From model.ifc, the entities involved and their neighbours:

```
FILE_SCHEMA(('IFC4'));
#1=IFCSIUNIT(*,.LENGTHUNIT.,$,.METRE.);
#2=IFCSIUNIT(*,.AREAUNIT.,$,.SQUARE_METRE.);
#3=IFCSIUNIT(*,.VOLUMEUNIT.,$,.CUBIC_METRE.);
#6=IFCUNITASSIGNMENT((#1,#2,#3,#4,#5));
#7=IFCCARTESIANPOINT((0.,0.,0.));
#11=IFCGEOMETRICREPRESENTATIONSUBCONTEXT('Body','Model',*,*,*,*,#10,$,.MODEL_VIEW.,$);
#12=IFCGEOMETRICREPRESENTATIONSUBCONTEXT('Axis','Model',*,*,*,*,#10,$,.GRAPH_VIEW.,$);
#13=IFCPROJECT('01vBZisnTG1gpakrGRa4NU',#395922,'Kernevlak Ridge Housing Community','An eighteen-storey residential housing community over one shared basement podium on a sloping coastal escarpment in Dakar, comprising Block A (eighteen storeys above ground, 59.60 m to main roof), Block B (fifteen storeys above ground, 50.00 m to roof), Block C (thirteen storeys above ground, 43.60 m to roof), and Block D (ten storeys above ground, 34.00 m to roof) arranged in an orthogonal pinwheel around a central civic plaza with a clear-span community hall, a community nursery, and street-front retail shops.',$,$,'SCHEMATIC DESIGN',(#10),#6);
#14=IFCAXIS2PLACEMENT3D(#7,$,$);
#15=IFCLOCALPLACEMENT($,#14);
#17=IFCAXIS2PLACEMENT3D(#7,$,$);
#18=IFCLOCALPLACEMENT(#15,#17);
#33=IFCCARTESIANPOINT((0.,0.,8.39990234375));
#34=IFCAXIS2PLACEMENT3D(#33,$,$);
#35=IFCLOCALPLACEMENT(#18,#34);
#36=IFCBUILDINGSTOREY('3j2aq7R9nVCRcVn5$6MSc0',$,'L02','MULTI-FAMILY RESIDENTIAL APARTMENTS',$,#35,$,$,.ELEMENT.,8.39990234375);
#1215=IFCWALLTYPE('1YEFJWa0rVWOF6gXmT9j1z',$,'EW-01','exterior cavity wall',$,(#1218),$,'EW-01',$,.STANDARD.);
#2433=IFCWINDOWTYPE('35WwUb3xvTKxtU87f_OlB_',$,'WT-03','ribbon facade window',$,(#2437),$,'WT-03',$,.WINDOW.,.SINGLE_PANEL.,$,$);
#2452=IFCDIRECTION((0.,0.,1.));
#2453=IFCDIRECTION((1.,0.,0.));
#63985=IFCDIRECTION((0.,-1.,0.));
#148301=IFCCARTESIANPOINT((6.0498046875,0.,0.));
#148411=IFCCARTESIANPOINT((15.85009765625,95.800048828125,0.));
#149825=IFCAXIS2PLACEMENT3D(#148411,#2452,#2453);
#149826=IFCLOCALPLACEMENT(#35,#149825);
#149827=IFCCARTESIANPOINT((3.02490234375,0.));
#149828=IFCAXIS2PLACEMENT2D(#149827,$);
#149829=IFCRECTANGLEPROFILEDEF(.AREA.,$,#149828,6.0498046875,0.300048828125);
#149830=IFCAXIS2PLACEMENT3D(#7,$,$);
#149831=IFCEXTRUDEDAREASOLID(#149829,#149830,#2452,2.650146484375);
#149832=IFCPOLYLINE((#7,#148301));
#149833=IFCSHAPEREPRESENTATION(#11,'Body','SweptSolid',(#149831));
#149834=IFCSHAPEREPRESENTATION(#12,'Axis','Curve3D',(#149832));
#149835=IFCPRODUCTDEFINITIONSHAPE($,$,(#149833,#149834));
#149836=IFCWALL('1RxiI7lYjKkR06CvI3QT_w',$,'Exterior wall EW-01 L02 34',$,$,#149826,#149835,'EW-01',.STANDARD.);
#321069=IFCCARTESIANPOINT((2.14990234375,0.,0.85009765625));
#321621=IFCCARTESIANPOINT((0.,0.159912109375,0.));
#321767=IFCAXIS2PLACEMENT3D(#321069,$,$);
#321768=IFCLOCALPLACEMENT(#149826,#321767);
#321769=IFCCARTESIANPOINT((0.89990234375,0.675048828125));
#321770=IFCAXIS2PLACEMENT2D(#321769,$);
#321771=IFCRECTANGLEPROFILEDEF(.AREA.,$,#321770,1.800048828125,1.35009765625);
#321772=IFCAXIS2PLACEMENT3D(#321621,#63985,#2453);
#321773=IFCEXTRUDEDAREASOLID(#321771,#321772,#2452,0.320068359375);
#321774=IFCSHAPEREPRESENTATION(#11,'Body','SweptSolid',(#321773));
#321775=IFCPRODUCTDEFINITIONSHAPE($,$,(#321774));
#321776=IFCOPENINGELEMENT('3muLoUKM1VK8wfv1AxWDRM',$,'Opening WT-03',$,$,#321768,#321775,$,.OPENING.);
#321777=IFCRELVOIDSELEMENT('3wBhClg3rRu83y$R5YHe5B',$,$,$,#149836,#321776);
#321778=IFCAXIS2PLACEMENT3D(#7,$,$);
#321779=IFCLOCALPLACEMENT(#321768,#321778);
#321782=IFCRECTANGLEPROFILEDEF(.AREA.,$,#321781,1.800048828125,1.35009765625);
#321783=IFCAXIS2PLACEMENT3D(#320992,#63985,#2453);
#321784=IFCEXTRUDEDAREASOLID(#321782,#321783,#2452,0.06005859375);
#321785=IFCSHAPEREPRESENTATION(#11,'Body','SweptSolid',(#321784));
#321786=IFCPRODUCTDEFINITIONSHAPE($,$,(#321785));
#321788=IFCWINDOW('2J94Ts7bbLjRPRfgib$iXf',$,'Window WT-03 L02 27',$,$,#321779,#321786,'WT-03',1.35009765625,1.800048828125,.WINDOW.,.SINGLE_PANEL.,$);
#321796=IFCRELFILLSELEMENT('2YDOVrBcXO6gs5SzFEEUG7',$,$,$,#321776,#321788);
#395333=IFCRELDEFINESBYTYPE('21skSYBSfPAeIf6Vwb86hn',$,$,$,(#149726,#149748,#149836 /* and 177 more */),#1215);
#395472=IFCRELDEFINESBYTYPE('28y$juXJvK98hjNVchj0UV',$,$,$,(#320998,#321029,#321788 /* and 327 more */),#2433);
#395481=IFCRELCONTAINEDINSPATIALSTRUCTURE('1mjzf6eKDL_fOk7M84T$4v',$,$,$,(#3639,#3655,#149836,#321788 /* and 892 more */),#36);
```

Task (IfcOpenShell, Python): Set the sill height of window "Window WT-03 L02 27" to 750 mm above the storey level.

```python
import numpy as np
import ifcopenshell
import ifcopenshell.api.geometry
import ifcopenshell.geom
import ifcopenshell.util.element
import ifcopenshell.util.placement
import ifcopenshell.util.shape
import ifcopenshell.util.unit

model = ifcopenshell.open("model.ifc")
unit_scale = ifcopenshell.util.unit.calculate_unit_scale(model)

window = model.by_guid("2J94Ts7bbLjRPRfgib$iXf")
opening = window.FillsVoids[0].RelatingOpeningElement
storey = ifcopenshell.util.element.get_container(window, ifc_class="IfcBuildingStorey")
level = ifcopenshell.util.placement.get_local_placement(storey.ObjectPlacement)[2, 3]

# The opening's origin need not be at the sill, so measure its lowest point.
shape = ifcopenshell.geom.create_shape(ifcopenshell.geom.settings(), opening)
bottom = ifcopenshell.util.shape.get_shape_bottom_elevation(shape, shape.geometry) / unit_scale
dz = level + 0.75 - bottom

shift = np.array([0.0, 0.0, dz])
# The window is placed relative to its opening, so it follows when the opening moves.
matrix = ifcopenshell.util.placement.get_local_placement(opening.ObjectPlacement)
matrix[:3, 3] += shift
ifcopenshell.api.geometry.edit_object_placement(
    model, product=opening, matrix=matrix, is_si=False, should_transform_children=True
)

print(f"moved by {dz * unit_scale:+.3f} m")

model.write("model_rev.ifc")
```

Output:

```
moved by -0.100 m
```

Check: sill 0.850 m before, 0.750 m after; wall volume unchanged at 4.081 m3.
